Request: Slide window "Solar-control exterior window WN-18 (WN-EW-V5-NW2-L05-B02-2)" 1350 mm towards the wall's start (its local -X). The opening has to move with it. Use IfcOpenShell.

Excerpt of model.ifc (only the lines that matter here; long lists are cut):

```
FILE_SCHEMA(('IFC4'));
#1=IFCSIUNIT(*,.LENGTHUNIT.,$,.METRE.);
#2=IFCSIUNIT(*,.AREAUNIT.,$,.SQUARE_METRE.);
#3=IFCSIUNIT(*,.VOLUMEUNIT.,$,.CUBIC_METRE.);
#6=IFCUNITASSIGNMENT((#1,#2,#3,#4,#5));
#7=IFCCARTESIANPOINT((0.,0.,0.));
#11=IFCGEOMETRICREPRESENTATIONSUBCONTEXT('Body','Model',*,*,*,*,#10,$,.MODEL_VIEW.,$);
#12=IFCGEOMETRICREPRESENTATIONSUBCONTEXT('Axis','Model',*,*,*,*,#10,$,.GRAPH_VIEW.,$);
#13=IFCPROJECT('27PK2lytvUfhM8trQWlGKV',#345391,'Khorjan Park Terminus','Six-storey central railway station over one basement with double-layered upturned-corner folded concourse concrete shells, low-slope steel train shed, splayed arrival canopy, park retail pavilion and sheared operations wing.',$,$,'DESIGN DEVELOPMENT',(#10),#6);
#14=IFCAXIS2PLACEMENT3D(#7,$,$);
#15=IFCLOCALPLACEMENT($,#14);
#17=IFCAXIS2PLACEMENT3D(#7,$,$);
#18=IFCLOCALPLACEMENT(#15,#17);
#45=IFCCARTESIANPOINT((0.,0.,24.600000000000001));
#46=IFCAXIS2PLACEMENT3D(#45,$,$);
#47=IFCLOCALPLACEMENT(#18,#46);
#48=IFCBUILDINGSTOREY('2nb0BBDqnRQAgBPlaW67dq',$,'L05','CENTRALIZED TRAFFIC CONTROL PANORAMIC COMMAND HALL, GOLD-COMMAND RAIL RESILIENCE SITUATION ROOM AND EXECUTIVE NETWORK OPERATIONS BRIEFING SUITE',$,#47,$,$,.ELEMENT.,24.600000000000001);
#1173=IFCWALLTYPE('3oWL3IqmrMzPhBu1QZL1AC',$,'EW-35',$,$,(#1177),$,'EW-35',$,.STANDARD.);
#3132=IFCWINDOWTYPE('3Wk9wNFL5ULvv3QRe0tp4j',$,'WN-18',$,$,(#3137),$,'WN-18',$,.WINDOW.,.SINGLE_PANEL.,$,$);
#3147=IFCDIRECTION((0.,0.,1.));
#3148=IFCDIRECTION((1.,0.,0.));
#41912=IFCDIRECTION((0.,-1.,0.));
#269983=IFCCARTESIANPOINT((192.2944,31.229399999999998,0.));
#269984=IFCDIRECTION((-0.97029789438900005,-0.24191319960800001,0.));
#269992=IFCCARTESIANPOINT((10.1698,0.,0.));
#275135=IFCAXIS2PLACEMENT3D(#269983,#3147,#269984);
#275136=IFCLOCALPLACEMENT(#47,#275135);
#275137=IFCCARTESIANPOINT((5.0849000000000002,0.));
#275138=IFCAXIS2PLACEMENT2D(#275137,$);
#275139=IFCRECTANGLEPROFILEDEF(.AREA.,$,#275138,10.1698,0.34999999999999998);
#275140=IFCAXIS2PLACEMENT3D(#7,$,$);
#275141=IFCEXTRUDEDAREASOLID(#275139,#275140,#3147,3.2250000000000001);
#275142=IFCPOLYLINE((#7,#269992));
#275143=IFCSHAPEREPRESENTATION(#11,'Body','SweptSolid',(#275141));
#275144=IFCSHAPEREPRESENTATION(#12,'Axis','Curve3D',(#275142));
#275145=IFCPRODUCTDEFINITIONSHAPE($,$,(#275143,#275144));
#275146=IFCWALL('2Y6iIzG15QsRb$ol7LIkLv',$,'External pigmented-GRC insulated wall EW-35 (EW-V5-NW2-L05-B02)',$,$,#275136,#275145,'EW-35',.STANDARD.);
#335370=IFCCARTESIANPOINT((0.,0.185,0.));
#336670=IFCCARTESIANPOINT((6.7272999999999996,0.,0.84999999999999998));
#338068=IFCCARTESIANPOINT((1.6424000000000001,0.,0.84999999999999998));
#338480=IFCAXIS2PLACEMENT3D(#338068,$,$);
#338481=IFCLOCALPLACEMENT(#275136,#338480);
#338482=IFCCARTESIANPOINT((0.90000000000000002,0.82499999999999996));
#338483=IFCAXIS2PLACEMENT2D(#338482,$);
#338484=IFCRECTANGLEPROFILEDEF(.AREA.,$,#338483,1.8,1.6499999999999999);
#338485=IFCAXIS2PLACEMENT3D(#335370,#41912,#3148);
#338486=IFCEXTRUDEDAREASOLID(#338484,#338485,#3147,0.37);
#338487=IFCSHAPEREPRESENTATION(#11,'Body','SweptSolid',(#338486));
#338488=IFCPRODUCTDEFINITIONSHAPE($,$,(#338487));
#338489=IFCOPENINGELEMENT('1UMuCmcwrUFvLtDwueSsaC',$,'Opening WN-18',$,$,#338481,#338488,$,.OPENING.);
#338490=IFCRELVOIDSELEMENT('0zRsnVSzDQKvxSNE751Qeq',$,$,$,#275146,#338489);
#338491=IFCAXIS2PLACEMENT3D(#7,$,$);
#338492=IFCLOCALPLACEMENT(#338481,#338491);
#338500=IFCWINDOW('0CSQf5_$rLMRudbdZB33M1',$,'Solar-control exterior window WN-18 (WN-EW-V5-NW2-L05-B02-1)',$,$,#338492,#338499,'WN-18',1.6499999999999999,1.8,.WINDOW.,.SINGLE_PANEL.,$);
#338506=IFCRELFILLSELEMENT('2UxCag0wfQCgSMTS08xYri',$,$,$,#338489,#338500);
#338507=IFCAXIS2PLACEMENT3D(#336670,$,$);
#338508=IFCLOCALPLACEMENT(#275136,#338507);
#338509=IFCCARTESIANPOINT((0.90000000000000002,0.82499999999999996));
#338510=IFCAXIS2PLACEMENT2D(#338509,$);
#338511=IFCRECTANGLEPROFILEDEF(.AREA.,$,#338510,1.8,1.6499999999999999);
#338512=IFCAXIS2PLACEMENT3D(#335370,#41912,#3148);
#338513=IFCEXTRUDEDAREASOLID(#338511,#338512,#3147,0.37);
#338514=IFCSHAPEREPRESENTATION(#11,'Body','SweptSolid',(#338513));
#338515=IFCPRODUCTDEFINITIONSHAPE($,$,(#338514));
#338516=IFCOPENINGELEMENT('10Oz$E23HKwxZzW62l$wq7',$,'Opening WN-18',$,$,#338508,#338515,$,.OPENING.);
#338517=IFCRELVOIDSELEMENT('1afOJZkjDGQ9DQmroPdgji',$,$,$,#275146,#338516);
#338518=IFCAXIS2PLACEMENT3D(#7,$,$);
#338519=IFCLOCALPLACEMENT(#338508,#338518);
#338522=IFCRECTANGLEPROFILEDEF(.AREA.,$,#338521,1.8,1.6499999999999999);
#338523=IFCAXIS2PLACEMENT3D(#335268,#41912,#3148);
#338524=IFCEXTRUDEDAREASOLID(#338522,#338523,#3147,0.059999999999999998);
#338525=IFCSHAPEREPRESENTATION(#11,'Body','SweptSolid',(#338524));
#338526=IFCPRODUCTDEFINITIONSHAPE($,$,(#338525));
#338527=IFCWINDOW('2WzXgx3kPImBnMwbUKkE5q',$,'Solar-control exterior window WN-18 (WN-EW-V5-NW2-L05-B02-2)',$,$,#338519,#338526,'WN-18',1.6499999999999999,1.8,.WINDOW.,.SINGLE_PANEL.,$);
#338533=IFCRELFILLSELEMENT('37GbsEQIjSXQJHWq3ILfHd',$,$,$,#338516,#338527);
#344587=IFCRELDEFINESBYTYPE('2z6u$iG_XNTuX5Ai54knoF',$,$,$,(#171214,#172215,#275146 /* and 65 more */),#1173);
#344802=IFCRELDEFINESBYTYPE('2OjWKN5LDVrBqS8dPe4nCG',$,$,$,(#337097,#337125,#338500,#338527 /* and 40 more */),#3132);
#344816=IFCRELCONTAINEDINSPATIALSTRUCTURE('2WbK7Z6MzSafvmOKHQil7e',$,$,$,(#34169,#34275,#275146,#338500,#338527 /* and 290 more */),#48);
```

```python
import ifcopenshell
import ifcopenshell.api.geometry
import ifcopenshell.util.placement
import ifcopenshell.util.unit

model = ifcopenshell.open("model.ifc")
unit_scale = ifcopenshell.util.unit.calculate_unit_scale(model)

window = model.by_guid("2WzXgx3kPImBnMwbUKkE5q")
opening = window.FillsVoids[0].RelatingOpeningElement
wall = opening.VoidsElements[0].RelatingBuildingElement

wall_matrix = ifcopenshell.util.placement.get_local_placement(wall.ObjectPlacement)
shift = wall_matrix[:3, 0] * -1.35 / unit_scale
before = ifcopenshell.util.placement.get_local_placement(window.ObjectPlacement)[:3, 3].copy()

# The window is placed relative to its opening, so it follows when the opening moves.
matrix = ifcopenshell.util.placement.get_local_placement(opening.ObjectPlacement)
matrix[:3, 3] += shift
ifcopenshell.api.geometry.edit_object_placement(
    model, product=opening, matrix=matrix, is_si=False, should_transform_children=True
)

after = ifcopenshell.util.placement.get_local_placement(window.ObjectPlacement)[:3, 3]
print("window moved by", (after - before).round(3) + 0.0)

model.write("model_v2.ifc")
```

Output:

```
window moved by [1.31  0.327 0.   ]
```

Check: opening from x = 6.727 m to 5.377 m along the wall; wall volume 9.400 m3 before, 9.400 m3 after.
